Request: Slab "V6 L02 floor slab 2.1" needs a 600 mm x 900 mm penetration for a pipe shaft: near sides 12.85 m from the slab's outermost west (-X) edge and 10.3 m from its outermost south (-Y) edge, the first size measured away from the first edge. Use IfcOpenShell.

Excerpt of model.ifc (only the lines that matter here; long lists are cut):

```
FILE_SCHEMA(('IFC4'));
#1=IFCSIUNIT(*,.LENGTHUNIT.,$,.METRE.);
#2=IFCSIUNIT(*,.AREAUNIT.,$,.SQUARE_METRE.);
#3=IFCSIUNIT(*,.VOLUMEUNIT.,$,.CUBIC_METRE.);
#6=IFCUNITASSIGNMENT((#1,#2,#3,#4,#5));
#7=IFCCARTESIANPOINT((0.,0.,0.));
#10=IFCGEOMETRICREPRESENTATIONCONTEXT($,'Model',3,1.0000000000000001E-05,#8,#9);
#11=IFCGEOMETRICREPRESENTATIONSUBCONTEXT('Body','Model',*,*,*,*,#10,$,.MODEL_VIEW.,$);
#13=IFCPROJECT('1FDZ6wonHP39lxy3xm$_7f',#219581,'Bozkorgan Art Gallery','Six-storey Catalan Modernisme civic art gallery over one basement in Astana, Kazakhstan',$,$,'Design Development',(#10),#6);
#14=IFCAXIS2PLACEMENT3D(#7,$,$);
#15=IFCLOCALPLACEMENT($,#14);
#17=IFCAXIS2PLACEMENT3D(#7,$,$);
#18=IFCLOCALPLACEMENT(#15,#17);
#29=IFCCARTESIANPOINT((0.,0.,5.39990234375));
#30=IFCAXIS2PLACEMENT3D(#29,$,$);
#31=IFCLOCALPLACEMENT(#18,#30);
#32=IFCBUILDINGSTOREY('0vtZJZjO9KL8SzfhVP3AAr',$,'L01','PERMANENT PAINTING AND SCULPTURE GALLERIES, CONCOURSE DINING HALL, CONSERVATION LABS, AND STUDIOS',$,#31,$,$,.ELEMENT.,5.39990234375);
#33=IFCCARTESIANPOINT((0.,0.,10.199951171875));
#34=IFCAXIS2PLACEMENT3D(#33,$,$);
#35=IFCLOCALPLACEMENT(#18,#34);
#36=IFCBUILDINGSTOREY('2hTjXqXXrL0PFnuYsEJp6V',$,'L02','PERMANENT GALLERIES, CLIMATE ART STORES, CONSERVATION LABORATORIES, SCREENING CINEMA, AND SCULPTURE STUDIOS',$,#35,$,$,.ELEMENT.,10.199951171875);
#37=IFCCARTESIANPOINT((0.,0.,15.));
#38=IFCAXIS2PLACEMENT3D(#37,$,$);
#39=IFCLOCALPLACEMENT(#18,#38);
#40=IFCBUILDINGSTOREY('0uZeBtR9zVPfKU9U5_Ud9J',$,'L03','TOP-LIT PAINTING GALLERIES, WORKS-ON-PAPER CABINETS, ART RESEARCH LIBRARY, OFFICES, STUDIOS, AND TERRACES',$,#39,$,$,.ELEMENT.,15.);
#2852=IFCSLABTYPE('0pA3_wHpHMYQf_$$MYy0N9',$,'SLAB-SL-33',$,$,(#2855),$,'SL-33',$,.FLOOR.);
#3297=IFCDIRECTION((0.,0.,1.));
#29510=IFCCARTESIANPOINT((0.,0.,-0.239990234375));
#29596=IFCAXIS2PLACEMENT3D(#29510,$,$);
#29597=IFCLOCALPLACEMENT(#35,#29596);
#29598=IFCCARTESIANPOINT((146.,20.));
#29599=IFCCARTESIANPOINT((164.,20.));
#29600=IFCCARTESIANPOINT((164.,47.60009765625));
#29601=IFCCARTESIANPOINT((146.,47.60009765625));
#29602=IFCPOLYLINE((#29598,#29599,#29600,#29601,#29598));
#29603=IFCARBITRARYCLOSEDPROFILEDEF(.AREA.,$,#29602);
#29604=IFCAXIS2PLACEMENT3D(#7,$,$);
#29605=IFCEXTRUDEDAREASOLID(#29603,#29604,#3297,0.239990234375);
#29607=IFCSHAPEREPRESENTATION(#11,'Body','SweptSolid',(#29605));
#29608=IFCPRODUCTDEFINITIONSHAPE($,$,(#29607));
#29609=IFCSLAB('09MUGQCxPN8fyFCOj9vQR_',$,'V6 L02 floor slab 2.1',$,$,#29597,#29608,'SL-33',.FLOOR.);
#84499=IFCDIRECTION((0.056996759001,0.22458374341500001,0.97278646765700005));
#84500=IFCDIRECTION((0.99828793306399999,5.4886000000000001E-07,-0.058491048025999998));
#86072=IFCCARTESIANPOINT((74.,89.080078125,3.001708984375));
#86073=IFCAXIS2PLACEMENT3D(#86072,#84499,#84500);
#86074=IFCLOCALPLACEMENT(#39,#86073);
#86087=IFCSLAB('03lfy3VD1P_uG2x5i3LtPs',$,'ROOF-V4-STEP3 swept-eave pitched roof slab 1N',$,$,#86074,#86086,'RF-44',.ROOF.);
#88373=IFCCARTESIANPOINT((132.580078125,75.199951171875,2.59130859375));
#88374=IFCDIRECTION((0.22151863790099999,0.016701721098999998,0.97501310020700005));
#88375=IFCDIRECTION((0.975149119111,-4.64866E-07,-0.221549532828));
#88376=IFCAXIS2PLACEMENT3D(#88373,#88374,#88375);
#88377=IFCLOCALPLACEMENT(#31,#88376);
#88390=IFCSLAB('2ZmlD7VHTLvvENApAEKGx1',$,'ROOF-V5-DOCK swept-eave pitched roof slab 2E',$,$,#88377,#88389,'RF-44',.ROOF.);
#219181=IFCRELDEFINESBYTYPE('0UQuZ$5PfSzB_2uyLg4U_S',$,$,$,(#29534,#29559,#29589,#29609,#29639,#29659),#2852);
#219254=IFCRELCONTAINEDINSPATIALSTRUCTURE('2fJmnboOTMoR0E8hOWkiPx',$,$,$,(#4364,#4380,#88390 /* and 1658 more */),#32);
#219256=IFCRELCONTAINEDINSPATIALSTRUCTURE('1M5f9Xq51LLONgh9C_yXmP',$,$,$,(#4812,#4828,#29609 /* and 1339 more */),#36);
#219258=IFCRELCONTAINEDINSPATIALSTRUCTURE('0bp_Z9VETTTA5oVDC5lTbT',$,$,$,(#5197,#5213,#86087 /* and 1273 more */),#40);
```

```python
import numpy as np
import ifcopenshell
import ifcopenshell.api.feature
import ifcopenshell.api.geometry
import ifcopenshell.api.root
import ifcopenshell.geom
import ifcopenshell.util.placement
import ifcopenshell.util.representation
import ifcopenshell.util.shape
import ifcopenshell.util.unit

model = ifcopenshell.open("model.ifc")
unit_scale = ifcopenshell.util.unit.calculate_unit_scale(model)
settings = ifcopenshell.geom.settings()


def volume(element):
    """Net volume in cubic metres, openings subtracted."""
    shape = ifcopenshell.geom.create_shape(settings, element)
    return ifcopenshell.util.shape.get_volume(shape.geometry)


slab = model.by_guid("09MUGQCxPN8fyFCOj9vQR_")
before = volume(slab)

# Extent in the slab's own axes, in metres. The edges named are its -X and -Y sides.
slab_shape = ifcopenshell.geom.create_shape(settings, slab)
vertices = ifcopenshell.util.shape.get_vertices(slab_shape.geometry)
x_min, y_min, bottom = vertices.min(axis=0)
top = vertices[:, 2].max()

opening = ifcopenshell.api.root.create_entity(model, ifc_class="IfcOpeningElement", name="Pipe shaft opening", predefined_type="OPENING")
context = ifcopenshell.util.representation.get_context(model, "Model", "Body", "MODEL_VIEW")
width, depth = 0.6, 0.9
outline = [(0.0, 0.0), (width, 0.0), (width, depth), (0.0, depth), (0.0, 0.0)]
# Overshoot both faces by 50 mm so the cut is clean.
shape = ifcopenshell.api.geometry.add_slab_representation(
    model, context=context, depth=top - bottom + 0.1, polyline=outline
)
ifcopenshell.api.geometry.assign_representation(model, product=opening, representation=shape)

matrix = ifcopenshell.util.placement.get_local_placement(slab.ObjectPlacement)
matrix[:, 3] = matrix @ np.append(np.array([x_min + 12.85, y_min + 10.3, bottom - 0.05]) / unit_scale, 1.0)
ifcopenshell.api.geometry.edit_object_placement(model, product=opening, matrix=matrix, is_si=False)
ifcopenshell.api.feature.add_feature(model, feature=opening, element=slab)

after = volume(slab)

print(f"slab volume {before:.3f} -> {after:.3f} m3")

model.write("model_edited.ifc")
```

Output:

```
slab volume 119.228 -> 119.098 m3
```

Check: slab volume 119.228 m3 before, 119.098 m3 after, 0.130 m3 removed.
